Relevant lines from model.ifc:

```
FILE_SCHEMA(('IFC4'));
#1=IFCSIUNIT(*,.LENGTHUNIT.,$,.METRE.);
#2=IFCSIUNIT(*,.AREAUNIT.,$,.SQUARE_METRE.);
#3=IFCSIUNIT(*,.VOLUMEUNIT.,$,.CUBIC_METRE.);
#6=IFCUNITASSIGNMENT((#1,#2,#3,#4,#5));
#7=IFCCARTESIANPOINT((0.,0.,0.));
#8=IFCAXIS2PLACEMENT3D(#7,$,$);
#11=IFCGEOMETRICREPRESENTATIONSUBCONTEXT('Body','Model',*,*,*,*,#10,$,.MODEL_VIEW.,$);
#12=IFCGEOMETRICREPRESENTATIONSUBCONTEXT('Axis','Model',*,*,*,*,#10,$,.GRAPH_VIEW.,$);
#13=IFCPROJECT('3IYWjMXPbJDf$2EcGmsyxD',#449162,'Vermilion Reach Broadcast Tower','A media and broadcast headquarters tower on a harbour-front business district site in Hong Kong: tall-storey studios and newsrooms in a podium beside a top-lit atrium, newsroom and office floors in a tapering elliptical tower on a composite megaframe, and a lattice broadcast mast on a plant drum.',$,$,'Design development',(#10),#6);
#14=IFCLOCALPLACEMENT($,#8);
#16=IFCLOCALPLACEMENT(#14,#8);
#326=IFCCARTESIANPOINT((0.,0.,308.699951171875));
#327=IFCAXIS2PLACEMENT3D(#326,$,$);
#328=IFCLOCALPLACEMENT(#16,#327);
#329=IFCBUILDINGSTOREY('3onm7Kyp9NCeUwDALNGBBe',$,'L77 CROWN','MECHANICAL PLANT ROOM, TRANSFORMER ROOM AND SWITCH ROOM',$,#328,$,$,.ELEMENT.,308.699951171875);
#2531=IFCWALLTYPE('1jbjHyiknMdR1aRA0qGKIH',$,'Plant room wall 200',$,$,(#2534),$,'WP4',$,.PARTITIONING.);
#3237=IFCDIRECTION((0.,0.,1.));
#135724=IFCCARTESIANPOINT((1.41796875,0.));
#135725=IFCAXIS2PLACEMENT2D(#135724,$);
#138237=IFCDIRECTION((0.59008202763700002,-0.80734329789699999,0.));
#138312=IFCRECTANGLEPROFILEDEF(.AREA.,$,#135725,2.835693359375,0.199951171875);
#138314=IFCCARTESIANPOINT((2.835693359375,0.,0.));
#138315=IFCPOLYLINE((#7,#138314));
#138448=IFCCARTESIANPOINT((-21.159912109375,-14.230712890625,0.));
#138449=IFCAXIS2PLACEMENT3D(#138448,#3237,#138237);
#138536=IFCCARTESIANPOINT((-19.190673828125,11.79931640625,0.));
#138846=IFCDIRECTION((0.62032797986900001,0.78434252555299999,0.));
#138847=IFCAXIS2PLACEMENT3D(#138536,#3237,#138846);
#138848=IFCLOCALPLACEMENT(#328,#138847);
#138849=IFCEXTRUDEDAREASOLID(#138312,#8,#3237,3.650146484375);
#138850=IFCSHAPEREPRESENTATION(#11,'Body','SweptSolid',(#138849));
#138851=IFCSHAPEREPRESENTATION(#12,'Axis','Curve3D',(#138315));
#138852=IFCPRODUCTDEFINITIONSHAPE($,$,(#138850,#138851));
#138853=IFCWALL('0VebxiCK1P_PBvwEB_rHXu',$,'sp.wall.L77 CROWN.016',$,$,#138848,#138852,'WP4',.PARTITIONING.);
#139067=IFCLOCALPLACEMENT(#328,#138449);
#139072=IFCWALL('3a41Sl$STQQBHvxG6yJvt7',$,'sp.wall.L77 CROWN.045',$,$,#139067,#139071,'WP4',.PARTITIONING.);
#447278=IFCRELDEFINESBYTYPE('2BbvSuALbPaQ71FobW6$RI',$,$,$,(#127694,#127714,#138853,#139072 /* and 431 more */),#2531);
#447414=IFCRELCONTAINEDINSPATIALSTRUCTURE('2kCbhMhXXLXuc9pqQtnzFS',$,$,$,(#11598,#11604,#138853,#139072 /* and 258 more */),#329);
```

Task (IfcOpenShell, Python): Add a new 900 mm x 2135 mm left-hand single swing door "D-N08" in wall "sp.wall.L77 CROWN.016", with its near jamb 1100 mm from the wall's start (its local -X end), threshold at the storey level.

```python
import numpy as np
import ifcopenshell
import ifcopenshell.api.feature
import ifcopenshell.api.geometry
import ifcopenshell.api.root
import ifcopenshell.api.spatial
import ifcopenshell.geom
import ifcopenshell.util.element
import ifcopenshell.util.placement
import ifcopenshell.util.representation
import ifcopenshell.util.shape
import ifcopenshell.util.unit

model = ifcopenshell.open("model.ifc")
unit_scale = ifcopenshell.util.unit.calculate_unit_scale(model)
settings = ifcopenshell.geom.settings()


def volume(element):
    """Net volume in cubic metres, openings subtracted."""
    shape = ifcopenshell.geom.create_shape(settings, element)
    return ifcopenshell.util.shape.get_volume(shape.geometry)


wall = model.by_guid("0VebxiCK1P_PBvwEB_rHXu")
storey = ifcopenshell.util.element.get_container(wall, ifc_class="IfcBuildingStorey")
context = ifcopenshell.util.representation.get_context(model, "Model", "Body", "MODEL_VIEW")
before = volume(wall)

width, height, from_end, sill = 0.9, 2.135, 1.1, 0.0  # metres

# The wall runs along its own X axis, and the end named is its -X end.
wall_shape = ifcopenshell.geom.create_shape(settings, wall)
x, y, z = ifcopenshell.util.shape.get_vertices(wall_shape.geometry).T
start = x.min() + from_end
face, thickness = float(y.min()), float(y.max() - y.min())
wall_matrix = ifcopenshell.util.placement.get_local_placement(wall.ObjectPlacement)
level = ifcopenshell.util.placement.get_local_placement(storey.ObjectPlacement)[2, 3]


def in_wall(x, y):
    """Placement at x, y metres in the wall's axes, at sill height."""
    matrix = wall_matrix.copy()
    matrix[:, 3] = wall_matrix @ np.array([x / unit_scale, y / unit_scale, 0.0, 1.0])
    matrix[2, 3] = level + sill / unit_scale
    return matrix


# Opening: a box that overshoots both wall faces by 50 mm.
opening = ifcopenshell.api.root.create_entity(model, ifc_class="IfcOpeningElement", predefined_type="OPENING")
box = ifcopenshell.api.geometry.add_wall_representation(
    model, context=context, length=width, height=height, thickness=thickness + 0.1
)
ifcopenshell.api.geometry.assign_representation(model, product=opening, representation=box)
ifcopenshell.api.geometry.edit_object_placement(model, product=opening, matrix=in_wall(start, face - 0.05), is_si=False)
ifcopenshell.api.feature.add_feature(model, feature=opening, element=wall)

door = ifcopenshell.api.root.create_entity(model, ifc_class="IfcDoor", name="D-N08", predefined_type="DOOR")
door.OverallWidth, door.OverallHeight = width / unit_scale, height / unit_scale
door.OperationType = "SINGLE_SWING_LEFT"
body = ifcopenshell.api.geometry.add_door_representation(
    model,
    context=context,
    overall_width=door.OverallWidth,
    overall_height=door.OverallHeight,
    operation_type="SINGLE_SWING_LEFT",
    lining_properties={"LiningDepth": thickness / unit_scale, "ThresholdDepth": thickness / unit_scale},
)
ifcopenshell.api.geometry.assign_representation(model, product=door, representation=body)
ifcopenshell.api.spatial.assign_container(model, products=[door], relating_structure=storey)
ifcopenshell.api.feature.add_filling(model, opening=opening, element=door)

# The lining spans the wall, so the door starts at the wall face.
ifcopenshell.api.geometry.edit_object_placement(model, product=door, matrix=in_wall(start, face), is_si=False)

after = volume(wall)

print(f"wall volume {before:.3f} -> {after:.3f} m3")

model.write("model-out.ifc")
```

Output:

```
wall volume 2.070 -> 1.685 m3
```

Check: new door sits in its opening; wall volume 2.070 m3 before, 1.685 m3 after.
